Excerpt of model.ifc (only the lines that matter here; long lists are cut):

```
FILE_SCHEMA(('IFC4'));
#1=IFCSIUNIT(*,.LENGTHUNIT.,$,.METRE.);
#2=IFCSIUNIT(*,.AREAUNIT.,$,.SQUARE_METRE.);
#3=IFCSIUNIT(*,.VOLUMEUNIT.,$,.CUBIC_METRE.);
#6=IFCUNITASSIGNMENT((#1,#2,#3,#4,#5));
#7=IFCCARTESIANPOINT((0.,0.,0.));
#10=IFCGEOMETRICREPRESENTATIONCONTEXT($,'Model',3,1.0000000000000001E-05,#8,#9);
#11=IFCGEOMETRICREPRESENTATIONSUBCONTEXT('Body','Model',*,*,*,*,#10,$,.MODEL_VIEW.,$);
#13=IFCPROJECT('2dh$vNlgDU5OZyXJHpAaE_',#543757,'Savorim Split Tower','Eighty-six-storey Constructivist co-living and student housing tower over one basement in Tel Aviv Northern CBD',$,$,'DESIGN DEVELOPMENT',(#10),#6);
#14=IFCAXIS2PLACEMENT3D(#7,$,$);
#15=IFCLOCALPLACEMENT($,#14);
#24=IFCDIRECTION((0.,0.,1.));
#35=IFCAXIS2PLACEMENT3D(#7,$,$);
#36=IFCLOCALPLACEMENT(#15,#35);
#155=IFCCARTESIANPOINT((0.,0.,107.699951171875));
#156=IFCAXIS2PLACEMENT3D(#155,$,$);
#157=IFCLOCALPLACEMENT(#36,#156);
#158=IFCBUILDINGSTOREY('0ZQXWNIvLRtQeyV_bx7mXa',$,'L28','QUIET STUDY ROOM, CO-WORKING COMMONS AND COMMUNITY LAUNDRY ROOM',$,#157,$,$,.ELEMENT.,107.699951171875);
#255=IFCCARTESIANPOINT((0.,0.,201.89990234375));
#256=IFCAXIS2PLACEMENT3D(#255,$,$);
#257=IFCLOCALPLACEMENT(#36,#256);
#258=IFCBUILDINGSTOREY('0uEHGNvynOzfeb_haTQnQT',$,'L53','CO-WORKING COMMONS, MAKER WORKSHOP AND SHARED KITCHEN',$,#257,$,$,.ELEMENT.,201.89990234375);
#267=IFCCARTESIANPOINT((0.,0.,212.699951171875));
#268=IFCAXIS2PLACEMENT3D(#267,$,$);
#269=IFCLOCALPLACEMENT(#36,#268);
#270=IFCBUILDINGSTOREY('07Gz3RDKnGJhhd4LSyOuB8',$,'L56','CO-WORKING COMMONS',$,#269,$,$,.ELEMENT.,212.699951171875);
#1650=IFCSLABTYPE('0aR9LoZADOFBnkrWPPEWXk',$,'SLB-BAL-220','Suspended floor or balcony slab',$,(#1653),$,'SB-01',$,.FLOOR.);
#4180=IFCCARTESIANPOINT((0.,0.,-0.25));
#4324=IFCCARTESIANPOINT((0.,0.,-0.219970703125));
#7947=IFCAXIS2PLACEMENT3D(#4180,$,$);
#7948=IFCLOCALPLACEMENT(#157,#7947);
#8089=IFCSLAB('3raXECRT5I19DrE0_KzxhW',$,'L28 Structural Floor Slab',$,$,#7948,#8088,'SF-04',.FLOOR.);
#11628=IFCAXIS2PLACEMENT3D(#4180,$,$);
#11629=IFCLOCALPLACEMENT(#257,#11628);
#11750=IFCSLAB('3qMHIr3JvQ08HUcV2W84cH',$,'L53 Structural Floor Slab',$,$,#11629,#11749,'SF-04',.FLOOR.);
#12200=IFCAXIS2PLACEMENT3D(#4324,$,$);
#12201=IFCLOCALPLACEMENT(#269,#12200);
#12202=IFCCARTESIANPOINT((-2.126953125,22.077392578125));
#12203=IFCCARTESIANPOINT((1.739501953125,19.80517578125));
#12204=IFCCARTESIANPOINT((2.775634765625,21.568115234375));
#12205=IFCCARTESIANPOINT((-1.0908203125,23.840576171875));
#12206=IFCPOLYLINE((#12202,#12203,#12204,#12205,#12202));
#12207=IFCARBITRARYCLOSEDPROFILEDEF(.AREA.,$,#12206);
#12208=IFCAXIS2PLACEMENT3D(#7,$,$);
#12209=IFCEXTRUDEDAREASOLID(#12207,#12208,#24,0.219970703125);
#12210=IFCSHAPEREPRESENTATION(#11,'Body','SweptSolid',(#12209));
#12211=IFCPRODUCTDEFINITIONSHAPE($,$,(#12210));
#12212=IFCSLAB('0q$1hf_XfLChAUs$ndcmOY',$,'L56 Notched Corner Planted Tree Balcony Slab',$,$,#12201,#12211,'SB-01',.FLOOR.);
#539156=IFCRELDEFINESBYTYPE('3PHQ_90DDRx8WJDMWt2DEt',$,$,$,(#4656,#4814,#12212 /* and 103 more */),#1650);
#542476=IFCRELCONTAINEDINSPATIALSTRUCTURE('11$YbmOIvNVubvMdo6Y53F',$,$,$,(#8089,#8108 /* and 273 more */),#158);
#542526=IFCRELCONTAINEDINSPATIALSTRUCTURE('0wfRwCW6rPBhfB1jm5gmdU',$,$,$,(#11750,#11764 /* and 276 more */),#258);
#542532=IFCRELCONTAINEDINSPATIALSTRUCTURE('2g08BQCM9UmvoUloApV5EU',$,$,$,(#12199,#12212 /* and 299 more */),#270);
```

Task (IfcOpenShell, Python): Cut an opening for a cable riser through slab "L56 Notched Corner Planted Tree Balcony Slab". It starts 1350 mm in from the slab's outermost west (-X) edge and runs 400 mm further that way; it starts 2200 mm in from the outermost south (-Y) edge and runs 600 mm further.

```python
import numpy as np
import ifcopenshell
import ifcopenshell.api.feature
import ifcopenshell.api.geometry
import ifcopenshell.api.root
import ifcopenshell.geom
import ifcopenshell.util.placement
import ifcopenshell.util.representation
import ifcopenshell.util.shape
import ifcopenshell.util.unit

model = ifcopenshell.open("model.ifc")
unit_scale = ifcopenshell.util.unit.calculate_unit_scale(model)
settings = ifcopenshell.geom.settings()


def volume(element):
    """Net volume in cubic metres, openings subtracted."""
    shape = ifcopenshell.geom.create_shape(settings, element)
    return ifcopenshell.util.shape.get_volume(shape.geometry)


slab = model.by_guid("0q$1hf_XfLChAUs$ndcmOY")
before = volume(slab)

# Extent in the slab's own axes, in metres. The edges named are its -X and -Y sides.
slab_shape = ifcopenshell.geom.create_shape(settings, slab)
vertices = ifcopenshell.util.shape.get_vertices(slab_shape.geometry)
x_min, y_min, bottom = vertices.min(axis=0)
top = vertices[:, 2].max()

opening = ifcopenshell.api.root.create_entity(model, ifc_class="IfcOpeningElement", name="Cable riser opening", predefined_type="OPENING")
context = ifcopenshell.util.representation.get_context(model, "Model", "Body", "MODEL_VIEW")
width, depth = 0.4, 0.6
outline = [(0.0, 0.0), (width, 0.0), (width, depth), (0.0, depth), (0.0, 0.0)]
# Overshoot both faces by 50 mm so the cut is clean.
shape = ifcopenshell.api.geometry.add_slab_representation(
    model, context=context, depth=top - bottom + 0.1, polyline=outline
)
ifcopenshell.api.geometry.assign_representation(model, product=opening, representation=shape)

matrix = ifcopenshell.util.placement.get_local_placement(slab.ObjectPlacement)
matrix[:, 3] = matrix @ np.append(np.array([x_min + 1.35, y_min + 2.2, bottom - 0.05]) / unit_scale, 1.0)
ifcopenshell.api.geometry.edit_object_placement(model, product=opening, matrix=matrix, is_si=False)
ifcopenshell.api.feature.add_feature(model, feature=opening, element=slab)

after = volume(slab)

print(f"slab volume {before:.3f} -> {after:.3f} m3")

model.write("model-out.ifc")
```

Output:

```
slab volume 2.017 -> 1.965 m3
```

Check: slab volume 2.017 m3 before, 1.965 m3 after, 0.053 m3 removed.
